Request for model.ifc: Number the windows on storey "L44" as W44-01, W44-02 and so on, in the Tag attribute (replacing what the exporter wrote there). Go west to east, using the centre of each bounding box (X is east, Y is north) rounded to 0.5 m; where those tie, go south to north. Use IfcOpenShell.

First a look at what the model holds.

```python
import ifcopenshell
import ifcopenshell.util.element
import ifcopenshell.util.placement

model = ifcopenshell.open("model.ifc")
print(model.schema)
storey = next(s for s in model.by_type("IfcBuildingStorey") if s.Name == "L44")
windows = [e for e in ifcopenshell.util.element.get_decomposition(storey) if e.is_a("IfcWindow")]
for e in sorted(windows, key=lambda e: e.id()):
    origin = ifcopenshell.util.placement.get_local_placement(e.ObjectPlacement)[:3, 3]
    print(e.id(), e.Tag, e.Name, origin.round(2) + 0.0, sep=" | ")
```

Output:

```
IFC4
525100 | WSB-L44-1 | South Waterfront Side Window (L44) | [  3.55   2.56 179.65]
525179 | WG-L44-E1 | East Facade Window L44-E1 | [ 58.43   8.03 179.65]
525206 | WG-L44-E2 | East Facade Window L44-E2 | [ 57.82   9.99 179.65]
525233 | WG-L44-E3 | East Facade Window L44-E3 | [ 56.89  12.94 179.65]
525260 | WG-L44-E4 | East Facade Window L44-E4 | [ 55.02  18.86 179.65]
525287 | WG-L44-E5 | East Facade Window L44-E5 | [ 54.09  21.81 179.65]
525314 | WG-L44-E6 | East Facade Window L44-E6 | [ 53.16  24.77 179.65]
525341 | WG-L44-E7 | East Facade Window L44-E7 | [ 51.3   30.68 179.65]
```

```python
import ifcopenshell
import ifcopenshell.geom
import ifcopenshell.util.element
import ifcopenshell.util.shape

model = ifcopenshell.open("model.ifc")
settings = ifcopenshell.geom.settings()
settings.set("use-world-coords", True)


def centre(element):
    shape = ifcopenshell.geom.create_shape(settings, element)
    return ifcopenshell.util.shape.get_bbox_centroid(shape.geometry)


storey = next(s for s in model.by_type("IfcBuildingStorey") if s.Name == "L44")
windows = [e for e in ifcopenshell.util.element.get_decomposition(storey) if e.is_a("IfcWindow")]

# Insertion points can sit at a corner or the storey origin, so sort by the geometry (in metres).
centres = {e: centre(e) for e in windows}
windows.sort(key=lambda e: (round(centres[e][0] / 0.5), centres[e][1]))

for i, e in enumerate(windows, start=1):
    number = f"W44-{i:02d}"
    e.Tag = number
    print(e.id(), number)

model.write("model_v2.ifc")
```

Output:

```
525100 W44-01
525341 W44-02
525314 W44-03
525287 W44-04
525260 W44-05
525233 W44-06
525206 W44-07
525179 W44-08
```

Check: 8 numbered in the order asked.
